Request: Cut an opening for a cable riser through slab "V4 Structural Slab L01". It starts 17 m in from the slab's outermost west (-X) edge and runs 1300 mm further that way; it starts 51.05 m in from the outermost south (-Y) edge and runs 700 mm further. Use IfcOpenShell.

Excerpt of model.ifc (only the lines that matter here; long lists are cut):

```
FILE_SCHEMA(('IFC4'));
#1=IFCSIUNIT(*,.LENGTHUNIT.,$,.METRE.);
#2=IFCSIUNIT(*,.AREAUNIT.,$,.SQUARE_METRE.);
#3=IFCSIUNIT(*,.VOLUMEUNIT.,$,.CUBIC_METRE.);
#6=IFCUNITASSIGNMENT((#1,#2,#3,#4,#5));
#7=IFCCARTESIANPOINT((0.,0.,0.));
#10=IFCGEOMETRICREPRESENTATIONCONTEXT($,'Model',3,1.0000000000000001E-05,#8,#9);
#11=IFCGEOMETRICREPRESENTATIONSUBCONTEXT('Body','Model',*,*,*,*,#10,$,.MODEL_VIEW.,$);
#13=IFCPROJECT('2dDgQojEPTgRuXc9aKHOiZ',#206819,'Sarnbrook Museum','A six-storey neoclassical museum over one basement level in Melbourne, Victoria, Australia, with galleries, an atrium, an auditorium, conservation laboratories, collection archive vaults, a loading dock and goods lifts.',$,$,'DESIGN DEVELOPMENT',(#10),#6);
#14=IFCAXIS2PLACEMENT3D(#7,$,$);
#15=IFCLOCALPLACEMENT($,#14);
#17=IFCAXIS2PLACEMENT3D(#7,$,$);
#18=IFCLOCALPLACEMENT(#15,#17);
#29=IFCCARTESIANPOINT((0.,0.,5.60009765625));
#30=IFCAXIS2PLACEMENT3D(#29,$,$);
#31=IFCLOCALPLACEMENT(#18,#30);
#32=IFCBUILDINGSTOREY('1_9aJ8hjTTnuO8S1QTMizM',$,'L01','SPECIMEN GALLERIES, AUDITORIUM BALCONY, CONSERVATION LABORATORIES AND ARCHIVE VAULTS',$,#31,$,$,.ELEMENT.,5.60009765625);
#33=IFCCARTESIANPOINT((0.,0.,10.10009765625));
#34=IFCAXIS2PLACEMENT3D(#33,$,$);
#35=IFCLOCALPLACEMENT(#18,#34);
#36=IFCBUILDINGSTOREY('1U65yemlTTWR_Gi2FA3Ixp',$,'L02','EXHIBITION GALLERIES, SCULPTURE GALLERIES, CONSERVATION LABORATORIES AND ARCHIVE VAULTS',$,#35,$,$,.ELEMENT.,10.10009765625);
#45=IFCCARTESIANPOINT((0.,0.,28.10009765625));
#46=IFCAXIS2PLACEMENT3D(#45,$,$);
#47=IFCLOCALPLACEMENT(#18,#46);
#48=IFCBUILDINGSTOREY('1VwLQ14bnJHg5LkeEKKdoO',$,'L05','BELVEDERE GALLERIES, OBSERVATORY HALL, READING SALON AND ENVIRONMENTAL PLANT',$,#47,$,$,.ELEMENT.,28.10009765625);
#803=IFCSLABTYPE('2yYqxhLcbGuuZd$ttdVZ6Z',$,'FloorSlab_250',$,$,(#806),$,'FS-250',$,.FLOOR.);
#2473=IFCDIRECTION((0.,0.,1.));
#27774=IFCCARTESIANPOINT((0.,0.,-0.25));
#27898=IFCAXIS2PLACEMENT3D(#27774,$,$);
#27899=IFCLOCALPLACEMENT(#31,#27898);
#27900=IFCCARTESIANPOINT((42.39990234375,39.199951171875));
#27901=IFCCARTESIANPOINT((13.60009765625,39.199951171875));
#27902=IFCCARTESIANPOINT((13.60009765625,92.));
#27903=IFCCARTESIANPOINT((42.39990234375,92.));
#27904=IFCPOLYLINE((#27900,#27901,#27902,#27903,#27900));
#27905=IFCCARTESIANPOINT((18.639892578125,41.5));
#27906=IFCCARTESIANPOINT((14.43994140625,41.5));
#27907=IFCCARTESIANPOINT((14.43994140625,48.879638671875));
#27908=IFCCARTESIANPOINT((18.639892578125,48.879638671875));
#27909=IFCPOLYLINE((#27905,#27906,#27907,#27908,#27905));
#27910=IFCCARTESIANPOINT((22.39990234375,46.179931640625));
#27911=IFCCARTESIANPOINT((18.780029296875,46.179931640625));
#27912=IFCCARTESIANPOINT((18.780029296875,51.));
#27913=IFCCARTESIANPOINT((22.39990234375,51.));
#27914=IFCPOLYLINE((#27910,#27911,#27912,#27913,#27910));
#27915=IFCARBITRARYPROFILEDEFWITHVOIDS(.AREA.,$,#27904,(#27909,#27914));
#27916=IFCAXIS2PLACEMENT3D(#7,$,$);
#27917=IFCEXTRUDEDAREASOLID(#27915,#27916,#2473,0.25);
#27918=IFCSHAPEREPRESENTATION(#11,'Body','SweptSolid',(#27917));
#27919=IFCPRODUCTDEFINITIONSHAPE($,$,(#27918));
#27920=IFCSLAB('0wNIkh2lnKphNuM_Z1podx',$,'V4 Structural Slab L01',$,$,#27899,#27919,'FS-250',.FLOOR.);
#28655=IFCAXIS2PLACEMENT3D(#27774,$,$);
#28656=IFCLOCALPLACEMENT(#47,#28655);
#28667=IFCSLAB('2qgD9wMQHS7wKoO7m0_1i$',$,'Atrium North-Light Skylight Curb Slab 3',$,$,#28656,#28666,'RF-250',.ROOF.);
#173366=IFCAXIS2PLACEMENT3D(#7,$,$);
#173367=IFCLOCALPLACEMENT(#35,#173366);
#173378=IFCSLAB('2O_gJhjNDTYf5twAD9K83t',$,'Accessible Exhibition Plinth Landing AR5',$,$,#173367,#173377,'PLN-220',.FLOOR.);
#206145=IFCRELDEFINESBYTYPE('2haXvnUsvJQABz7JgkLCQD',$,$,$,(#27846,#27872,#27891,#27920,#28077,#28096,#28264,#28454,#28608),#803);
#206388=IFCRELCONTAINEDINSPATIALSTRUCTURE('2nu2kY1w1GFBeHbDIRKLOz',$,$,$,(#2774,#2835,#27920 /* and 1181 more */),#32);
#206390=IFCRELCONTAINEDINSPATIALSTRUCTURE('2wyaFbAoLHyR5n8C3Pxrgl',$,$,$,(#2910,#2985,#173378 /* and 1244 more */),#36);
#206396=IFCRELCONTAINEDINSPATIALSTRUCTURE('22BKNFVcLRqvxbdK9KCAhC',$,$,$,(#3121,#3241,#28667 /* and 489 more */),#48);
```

```python
import numpy as np
import ifcopenshell
import ifcopenshell.api.feature
import ifcopenshell.api.geometry
import ifcopenshell.api.root
import ifcopenshell.geom
import ifcopenshell.util.placement
import ifcopenshell.util.representation
import ifcopenshell.util.shape
import ifcopenshell.util.unit

model = ifcopenshell.open("model.ifc")
unit_scale = ifcopenshell.util.unit.calculate_unit_scale(model)
settings = ifcopenshell.geom.settings()


def volume(element):
    """Net volume in cubic metres, openings subtracted."""
    shape = ifcopenshell.geom.create_shape(settings, element)
    return ifcopenshell.util.shape.get_volume(shape.geometry)


slab = model.by_id(27920)
before = volume(slab)

# Extent in the slab's own axes, in metres. The edges named are its -X and -Y sides.
slab_shape = ifcopenshell.geom.create_shape(settings, slab)
vertices = ifcopenshell.util.shape.get_vertices(slab_shape.geometry)
x_min, y_min, bottom = vertices.min(axis=0)
top = vertices[:, 2].max()

opening = ifcopenshell.api.root.create_entity(model, ifc_class="IfcOpeningElement", name="Cable riser opening", predefined_type="OPENING")
context = ifcopenshell.util.representation.get_context(model, "Model", "Body", "MODEL_VIEW")
width, depth = 1.3, 0.7
outline = [(0.0, 0.0), (width, 0.0), (width, depth), (0.0, depth), (0.0, 0.0)]
# Overshoot both faces by 50 mm so the cut is clean.
shape = ifcopenshell.api.geometry.add_slab_representation(
    model, context=context, depth=top - bottom + 0.1, polyline=outline
)
ifcopenshell.api.geometry.assign_representation(model, product=opening, representation=shape)

matrix = ifcopenshell.util.placement.get_local_placement(slab.ObjectPlacement)
matrix[:, 3] = matrix @ np.append(np.array([x_min + 17, y_min + 51.05, bottom - 0.05]) / unit_scale, 1.0)
ifcopenshell.api.geometry.edit_object_placement(model, product=opening, matrix=matrix, is_si=False)
ifcopenshell.api.feature.add_feature(model, feature=opening, element=slab)

after = volume(slab)

print(f"slab volume {before:.3f} -> {after:.3f} m3")

model.write("model-out.ifc")
```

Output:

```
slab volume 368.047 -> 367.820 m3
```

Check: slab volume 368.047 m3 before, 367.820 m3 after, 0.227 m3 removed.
